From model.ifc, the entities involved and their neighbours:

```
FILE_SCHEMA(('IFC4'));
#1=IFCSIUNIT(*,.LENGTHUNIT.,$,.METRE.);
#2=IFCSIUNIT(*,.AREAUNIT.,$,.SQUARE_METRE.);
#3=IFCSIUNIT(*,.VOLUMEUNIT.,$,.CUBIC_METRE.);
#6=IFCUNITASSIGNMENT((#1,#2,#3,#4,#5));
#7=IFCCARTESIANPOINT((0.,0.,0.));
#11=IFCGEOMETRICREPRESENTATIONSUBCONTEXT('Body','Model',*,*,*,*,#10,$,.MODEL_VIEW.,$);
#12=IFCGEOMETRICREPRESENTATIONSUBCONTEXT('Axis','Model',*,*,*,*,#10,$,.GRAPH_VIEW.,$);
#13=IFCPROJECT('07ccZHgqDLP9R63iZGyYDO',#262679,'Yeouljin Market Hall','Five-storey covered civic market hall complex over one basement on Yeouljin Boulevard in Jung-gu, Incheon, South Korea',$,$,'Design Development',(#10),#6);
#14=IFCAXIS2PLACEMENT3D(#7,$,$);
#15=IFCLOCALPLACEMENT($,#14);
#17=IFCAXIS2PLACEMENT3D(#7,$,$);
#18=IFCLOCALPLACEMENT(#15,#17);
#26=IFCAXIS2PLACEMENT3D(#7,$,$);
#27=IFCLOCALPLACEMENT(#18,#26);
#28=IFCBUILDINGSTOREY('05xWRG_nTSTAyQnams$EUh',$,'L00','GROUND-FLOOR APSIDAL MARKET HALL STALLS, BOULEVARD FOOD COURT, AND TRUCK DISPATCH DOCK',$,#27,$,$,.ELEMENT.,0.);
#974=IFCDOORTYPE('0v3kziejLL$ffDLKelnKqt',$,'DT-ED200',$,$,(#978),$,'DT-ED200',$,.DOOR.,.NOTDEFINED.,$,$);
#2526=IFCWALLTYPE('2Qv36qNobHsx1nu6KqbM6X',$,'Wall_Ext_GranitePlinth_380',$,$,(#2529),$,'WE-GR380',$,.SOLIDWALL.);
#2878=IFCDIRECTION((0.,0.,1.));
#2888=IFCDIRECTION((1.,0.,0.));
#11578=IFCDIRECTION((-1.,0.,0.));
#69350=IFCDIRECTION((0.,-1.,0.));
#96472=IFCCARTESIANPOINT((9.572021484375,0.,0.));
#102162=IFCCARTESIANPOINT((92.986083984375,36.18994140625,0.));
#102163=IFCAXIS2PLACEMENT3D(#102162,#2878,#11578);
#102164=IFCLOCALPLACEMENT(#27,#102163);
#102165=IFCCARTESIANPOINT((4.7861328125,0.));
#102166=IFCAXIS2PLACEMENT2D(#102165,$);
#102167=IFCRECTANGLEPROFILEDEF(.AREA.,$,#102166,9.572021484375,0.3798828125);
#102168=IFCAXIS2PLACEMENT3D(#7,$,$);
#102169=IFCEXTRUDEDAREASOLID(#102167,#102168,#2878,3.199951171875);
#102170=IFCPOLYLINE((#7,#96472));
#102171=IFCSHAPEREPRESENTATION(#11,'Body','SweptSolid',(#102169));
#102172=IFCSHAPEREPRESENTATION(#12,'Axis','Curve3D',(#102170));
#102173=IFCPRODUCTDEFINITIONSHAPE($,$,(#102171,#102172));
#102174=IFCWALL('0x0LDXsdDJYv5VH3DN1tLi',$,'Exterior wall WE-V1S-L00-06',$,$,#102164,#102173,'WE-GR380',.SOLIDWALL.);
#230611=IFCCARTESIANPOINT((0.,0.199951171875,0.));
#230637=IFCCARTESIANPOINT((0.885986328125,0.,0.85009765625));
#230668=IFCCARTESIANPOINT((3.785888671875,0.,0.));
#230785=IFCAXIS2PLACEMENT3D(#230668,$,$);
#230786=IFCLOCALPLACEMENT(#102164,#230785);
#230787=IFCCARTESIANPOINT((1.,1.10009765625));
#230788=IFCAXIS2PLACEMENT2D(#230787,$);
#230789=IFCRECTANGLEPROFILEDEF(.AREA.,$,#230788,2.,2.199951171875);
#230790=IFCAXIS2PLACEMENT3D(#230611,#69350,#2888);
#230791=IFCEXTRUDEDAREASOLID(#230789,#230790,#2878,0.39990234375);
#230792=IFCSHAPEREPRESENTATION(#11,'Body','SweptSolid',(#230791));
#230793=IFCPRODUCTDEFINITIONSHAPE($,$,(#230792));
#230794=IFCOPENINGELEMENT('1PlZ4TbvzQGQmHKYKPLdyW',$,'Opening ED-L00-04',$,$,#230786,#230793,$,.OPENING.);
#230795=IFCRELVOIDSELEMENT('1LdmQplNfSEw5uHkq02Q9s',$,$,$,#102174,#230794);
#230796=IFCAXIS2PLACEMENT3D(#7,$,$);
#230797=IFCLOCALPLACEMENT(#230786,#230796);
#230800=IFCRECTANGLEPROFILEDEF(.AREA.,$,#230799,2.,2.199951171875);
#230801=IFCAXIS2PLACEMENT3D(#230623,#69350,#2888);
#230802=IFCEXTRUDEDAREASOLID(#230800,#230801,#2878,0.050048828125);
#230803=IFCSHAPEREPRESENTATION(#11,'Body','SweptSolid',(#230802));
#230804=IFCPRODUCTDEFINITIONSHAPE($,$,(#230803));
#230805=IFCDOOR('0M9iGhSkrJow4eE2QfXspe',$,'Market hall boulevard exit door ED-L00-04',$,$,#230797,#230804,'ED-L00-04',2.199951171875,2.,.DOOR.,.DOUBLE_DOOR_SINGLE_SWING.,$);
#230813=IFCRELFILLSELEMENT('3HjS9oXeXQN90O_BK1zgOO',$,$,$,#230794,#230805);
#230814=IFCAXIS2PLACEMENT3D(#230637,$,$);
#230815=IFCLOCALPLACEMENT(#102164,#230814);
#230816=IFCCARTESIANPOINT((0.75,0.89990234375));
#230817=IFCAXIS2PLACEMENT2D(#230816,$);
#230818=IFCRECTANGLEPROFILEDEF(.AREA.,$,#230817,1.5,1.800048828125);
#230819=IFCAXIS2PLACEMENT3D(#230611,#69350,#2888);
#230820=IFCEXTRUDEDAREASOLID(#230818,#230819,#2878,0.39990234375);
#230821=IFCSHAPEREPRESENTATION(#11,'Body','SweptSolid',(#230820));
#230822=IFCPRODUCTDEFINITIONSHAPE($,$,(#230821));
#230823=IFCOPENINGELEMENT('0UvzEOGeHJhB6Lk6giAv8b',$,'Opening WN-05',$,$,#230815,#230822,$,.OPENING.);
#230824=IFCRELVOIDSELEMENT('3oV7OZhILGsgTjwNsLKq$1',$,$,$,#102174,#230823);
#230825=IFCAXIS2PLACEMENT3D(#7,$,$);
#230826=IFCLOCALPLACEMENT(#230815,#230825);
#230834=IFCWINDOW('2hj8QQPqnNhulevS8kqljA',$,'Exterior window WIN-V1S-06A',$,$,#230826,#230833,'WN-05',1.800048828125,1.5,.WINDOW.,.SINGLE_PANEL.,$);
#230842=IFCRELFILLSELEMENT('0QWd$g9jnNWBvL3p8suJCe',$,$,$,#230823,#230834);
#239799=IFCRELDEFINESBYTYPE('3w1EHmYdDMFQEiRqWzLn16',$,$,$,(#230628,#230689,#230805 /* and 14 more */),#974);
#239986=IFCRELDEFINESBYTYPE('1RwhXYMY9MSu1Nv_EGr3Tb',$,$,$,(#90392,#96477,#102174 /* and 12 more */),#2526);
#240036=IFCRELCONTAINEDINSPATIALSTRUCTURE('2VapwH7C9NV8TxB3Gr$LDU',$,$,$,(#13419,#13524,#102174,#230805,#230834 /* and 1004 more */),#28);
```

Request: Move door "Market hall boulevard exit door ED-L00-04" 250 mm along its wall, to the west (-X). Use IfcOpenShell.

```python
import ifcopenshell
import ifcopenshell.api.geometry
import ifcopenshell.util.placement
import ifcopenshell.util.unit

model = ifcopenshell.open("model.ifc")
unit_scale = ifcopenshell.util.unit.calculate_unit_scale(model)

door = model.by_guid("0M9iGhSkrJow4eE2QfXspe")
opening = door.FillsVoids[0].RelatingOpeningElement
wall = opening.VoidsElements[0].RelatingBuildingElement

wall_matrix = ifcopenshell.util.placement.get_local_placement(wall.ObjectPlacement)
shift = wall_matrix[:3, 0] * 0.25 / unit_scale
before = ifcopenshell.util.placement.get_local_placement(door.ObjectPlacement)[:3, 3].copy()

# The door is placed relative to its opening, so it follows when the opening moves.
matrix = ifcopenshell.util.placement.get_local_placement(opening.ObjectPlacement)
matrix[:3, 3] += shift
ifcopenshell.api.geometry.edit_object_placement(
    model, product=opening, matrix=matrix, is_si=False, should_transform_children=True
)

after = ifcopenshell.util.placement.get_local_placement(door.ObjectPlacement)[:3, 3]
print("door moved by", (after - before).round(3) + 0.0)

model.write("model_edited.ifc")
```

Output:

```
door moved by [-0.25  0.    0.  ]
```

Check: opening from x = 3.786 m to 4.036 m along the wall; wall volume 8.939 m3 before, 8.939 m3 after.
